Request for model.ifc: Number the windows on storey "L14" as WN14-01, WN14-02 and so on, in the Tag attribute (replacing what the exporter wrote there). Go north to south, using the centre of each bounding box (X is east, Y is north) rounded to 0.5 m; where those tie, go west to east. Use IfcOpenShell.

First a look at what the model holds.

```python
import ifcopenshell
import ifcopenshell.util.element
import ifcopenshell.util.placement

model = ifcopenshell.open("model.ifc")
print(model.schema)
storey = next(s for s in model.by_type("IfcBuildingStorey") if s.Name == "L14")
windows = [e for e in ifcopenshell.util.element.get_decomposition(storey) if e.is_a("IfcWindow")]
for e in sorted(windows, key=lambda e: e.id()):
    origin = ifcopenshell.util.placement.get_local_placement(e.ObjectPlacement)[:3, 3]
    print(e.id(), e.Tag, e.Name, origin.round(2) + 0.0, sep=" | ")
```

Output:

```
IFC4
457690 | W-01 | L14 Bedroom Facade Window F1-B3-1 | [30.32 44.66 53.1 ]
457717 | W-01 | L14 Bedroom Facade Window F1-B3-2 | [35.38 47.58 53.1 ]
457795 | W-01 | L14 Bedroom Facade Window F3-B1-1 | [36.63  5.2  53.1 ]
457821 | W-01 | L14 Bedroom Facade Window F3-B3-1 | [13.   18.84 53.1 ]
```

```python
import ifcopenshell
import ifcopenshell.geom
import ifcopenshell.util.element
import ifcopenshell.util.shape

model = ifcopenshell.open("model.ifc")
settings = ifcopenshell.geom.settings()
settings.set("use-world-coords", True)


def centre(element):
    shape = ifcopenshell.geom.create_shape(settings, element)
    return ifcopenshell.util.shape.get_bbox_centroid(shape.geometry)


storey = next(s for s in model.by_type("IfcBuildingStorey") if s.Name == "L14")
windows = [e for e in ifcopenshell.util.element.get_decomposition(storey) if e.is_a("IfcWindow")]

# Insertion points can sit at a corner or the storey origin, so sort by the geometry (in metres).
centres = {e: centre(e) for e in windows}
windows.sort(key=lambda e: (-round(centres[e][1] / 0.5), centres[e][0]))

for i, e in enumerate(windows, start=1):
    number = f"WN14-{i:02d}"
    e.Tag = number
    print(e.id(), number)

model.write("model-out.ifc")
```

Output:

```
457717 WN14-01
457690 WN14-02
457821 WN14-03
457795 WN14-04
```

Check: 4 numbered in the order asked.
